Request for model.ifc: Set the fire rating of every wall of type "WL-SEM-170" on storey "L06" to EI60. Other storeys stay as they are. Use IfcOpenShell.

First a look at what the model holds.

```python
import ifcopenshell
import ifcopenshell.util.element

model = ifcopenshell.open("model.ifc")
print(model.schema)
storey = next(s for s in model.by_type("IfcBuildingStorey") if s.Name == "L06")
walls = [e for e in ifcopenshell.util.element.get_decomposition(storey) if e.is_a("IfcWall")]
seen = {}
for e in walls:
    element_type = ifcopenshell.util.element.get_type(e)
    key = (element_type.Name if element_type != e and element_type else None, ifcopenshell.util.element.get_pset(e, "Pset_WallCommon", "FireRating"))
    seen[key] = seen.get(key, 0) + 1
for (name, value), count in sorted(seen.items(), key=str):
    print(count, "x", name, "|", value)
```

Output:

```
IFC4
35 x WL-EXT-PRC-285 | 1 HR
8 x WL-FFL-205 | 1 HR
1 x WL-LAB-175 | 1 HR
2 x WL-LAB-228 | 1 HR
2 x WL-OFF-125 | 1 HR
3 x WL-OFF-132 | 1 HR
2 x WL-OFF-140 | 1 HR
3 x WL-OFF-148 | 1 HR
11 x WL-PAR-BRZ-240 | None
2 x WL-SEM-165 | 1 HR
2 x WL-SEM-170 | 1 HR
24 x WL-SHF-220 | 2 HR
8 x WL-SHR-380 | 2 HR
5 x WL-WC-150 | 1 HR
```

```python
import ifcopenshell
import ifcopenshell.api.pset
import ifcopenshell.util.element

model = ifcopenshell.open("model.ifc")

storey = next(s for s in model.by_type("IfcBuildingStorey") if s.Name == "L06")
walls = [e for e in ifcopenshell.util.element.get_decomposition(storey) if e.is_a("IfcWall")]

count = 0
for e in walls:
    element_type = ifcopenshell.util.element.get_type(e)
    if element_type in (None, e) or element_type.Name != "WL-SEM-170":
        continue
    # add_pset returns the element's existing set when there is one.
    pset = ifcopenshell.api.pset.add_pset(model, product=e, name="Pset_WallCommon")
    ifcopenshell.api.pset.edit_pset(model, pset=pset, properties={"FireRating": "EI60"})
    count += 1

print(count, "walls updated")

model.write("model_updated.ifc")
```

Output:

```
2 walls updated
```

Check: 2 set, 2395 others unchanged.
